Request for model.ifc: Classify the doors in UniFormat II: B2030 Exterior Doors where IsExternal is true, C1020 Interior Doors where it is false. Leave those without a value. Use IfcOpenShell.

First a look at what the model holds.

```python
import ifcopenshell
import ifcopenshell.util.element

model = ifcopenshell.open("model.ifc")
print(model.schema)
print("classifications:", [c.Name for c in model.by_type("IfcClassification")])
values = [ifcopenshell.util.element.get_pset(e, "Pset_DoorCommon", "IsExternal") for e in model.by_type("IfcDoor")]
for value in (True, False, None):
    print("IsExternal", value, values.count(value))
```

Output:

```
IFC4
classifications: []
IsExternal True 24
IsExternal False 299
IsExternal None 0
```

```python
import ifcopenshell
import ifcopenshell.api.classification
import ifcopenshell.util.element

model = ifcopenshell.open("model.ifc")

system = ifcopenshell.api.classification.add_classification(model, classification="UniFormat II")

doors = model.by_type("IfcDoor")
external = {e: ifcopenshell.util.element.get_pset(e, "Pset_DoorCommon", "IsExternal") for e in doors}
for flag, code, name in ((True, "B2030", "Exterior Doors"), (False, "C1020", "Interior Doors")):
    products = [e for e in doors if external[e] is flag]
    ifcopenshell.api.classification.add_reference(
        model, products=products, classification=system, identification=code, name=name
    )
    print(code, len(products))

model.write("model_updated.ifc")
```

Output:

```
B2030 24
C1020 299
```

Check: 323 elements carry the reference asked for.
